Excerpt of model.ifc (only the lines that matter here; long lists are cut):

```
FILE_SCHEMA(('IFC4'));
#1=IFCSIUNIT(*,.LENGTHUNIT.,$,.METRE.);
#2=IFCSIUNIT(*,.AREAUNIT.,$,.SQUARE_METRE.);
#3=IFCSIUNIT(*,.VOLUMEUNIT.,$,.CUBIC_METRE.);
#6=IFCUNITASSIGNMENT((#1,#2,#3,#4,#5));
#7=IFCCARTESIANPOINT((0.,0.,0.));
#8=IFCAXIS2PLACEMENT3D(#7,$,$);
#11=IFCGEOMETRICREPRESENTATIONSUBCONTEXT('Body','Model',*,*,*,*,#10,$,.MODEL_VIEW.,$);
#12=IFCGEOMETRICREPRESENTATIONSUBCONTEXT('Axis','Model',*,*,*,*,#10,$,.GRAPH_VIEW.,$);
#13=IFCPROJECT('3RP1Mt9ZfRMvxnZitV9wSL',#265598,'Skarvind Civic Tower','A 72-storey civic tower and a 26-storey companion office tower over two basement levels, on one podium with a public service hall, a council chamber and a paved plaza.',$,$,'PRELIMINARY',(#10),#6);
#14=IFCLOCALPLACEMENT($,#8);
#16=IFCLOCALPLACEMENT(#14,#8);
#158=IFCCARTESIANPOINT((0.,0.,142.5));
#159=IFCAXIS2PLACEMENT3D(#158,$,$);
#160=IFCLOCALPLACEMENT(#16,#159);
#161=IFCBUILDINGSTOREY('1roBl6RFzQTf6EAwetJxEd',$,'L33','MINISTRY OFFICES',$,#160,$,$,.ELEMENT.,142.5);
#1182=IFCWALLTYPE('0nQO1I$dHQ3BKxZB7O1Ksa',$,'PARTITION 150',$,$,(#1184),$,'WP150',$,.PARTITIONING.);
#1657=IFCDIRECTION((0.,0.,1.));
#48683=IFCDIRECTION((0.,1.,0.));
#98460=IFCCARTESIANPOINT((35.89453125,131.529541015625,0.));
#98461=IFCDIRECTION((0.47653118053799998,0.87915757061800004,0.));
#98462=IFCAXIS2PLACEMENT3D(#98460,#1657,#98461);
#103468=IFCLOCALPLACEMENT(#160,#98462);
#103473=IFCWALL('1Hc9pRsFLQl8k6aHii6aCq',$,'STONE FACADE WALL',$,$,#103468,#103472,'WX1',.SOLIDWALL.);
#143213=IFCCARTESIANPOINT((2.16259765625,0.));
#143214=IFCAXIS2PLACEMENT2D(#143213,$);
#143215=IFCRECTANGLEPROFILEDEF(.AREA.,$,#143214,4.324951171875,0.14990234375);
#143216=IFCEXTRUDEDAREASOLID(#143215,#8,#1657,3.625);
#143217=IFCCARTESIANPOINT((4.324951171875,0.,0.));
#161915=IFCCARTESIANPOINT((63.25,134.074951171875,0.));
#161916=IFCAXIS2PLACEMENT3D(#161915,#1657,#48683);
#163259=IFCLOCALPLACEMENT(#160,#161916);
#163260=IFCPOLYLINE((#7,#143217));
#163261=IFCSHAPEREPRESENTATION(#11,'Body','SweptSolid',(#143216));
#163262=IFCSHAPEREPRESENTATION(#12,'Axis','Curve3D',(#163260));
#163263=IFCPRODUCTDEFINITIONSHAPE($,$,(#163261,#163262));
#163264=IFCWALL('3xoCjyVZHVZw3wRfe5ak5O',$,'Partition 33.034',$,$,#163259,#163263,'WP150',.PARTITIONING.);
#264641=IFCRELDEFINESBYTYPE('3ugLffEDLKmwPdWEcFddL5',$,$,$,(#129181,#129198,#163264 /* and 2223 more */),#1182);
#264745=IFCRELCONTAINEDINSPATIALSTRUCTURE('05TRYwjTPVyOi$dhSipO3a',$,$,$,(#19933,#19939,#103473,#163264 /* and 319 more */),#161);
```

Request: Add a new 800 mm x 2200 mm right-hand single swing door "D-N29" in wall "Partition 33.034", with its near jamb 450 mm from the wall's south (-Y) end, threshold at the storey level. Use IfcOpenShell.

```python
import numpy as np
import ifcopenshell
import ifcopenshell.api.feature
import ifcopenshell.api.geometry
import ifcopenshell.api.root
import ifcopenshell.api.spatial
import ifcopenshell.geom
import ifcopenshell.util.element
import ifcopenshell.util.placement
import ifcopenshell.util.representation
import ifcopenshell.util.shape
import ifcopenshell.util.unit

model = ifcopenshell.open("model.ifc")
unit_scale = ifcopenshell.util.unit.calculate_unit_scale(model)
settings = ifcopenshell.geom.settings()


def volume(element):
    """Net volume in cubic metres, openings subtracted."""
    shape = ifcopenshell.geom.create_shape(settings, element)
    return ifcopenshell.util.shape.get_volume(shape.geometry)


wall = model.by_id(163264)
storey = ifcopenshell.util.element.get_container(wall, ifc_class="IfcBuildingStorey")
context = ifcopenshell.util.representation.get_context(model, "Model", "Body", "MODEL_VIEW")
before = volume(wall)

width, height, from_end, sill = 0.8, 2.2, 0.45, 0.0  # metres

# The wall runs along its own X axis, and the end named is its -X end.
wall_shape = ifcopenshell.geom.create_shape(settings, wall)
x, y, z = ifcopenshell.util.shape.get_vertices(wall_shape.geometry).T
start = x.min() + from_end
face, thickness = float(y.min()), float(y.max() - y.min())
wall_matrix = ifcopenshell.util.placement.get_local_placement(wall.ObjectPlacement)
level = ifcopenshell.util.placement.get_local_placement(storey.ObjectPlacement)[2, 3]


def in_wall(x, y):
    """Placement at x, y metres in the wall's axes, at sill height."""
    matrix = wall_matrix.copy()
    matrix[:, 3] = wall_matrix @ np.array([x / unit_scale, y / unit_scale, 0.0, 1.0])
    matrix[2, 3] = level + sill / unit_scale
    return matrix


# Opening: a box that overshoots both wall faces by 50 mm.
opening = ifcopenshell.api.root.create_entity(model, ifc_class="IfcOpeningElement", predefined_type="OPENING")
box = ifcopenshell.api.geometry.add_wall_representation(
    model, context=context, length=width, height=height, thickness=thickness + 0.1
)
ifcopenshell.api.geometry.assign_representation(model, product=opening, representation=box)
ifcopenshell.api.geometry.edit_object_placement(model, product=opening, matrix=in_wall(start, face - 0.05), is_si=False)
ifcopenshell.api.feature.add_feature(model, feature=opening, element=wall)

door = ifcopenshell.api.root.create_entity(model, ifc_class="IfcDoor", name="D-N29", predefined_type="DOOR")
door.OverallWidth, door.OverallHeight = width / unit_scale, height / unit_scale
door.OperationType = "SINGLE_SWING_RIGHT"
body = ifcopenshell.api.geometry.add_door_representation(
    model,
    context=context,
    overall_width=door.OverallWidth,
    overall_height=door.OverallHeight,
    operation_type="SINGLE_SWING_RIGHT",
    lining_properties={"LiningDepth": thickness / unit_scale, "ThresholdDepth": thickness / unit_scale},
)
ifcopenshell.api.geometry.assign_representation(model, product=door, representation=body)
ifcopenshell.api.spatial.assign_container(model, products=[door], relating_structure=storey)
ifcopenshell.api.feature.add_filling(model, opening=opening, element=door)

# The lining spans the wall, so the door starts at the wall face.
ifcopenshell.api.geometry.edit_object_placement(model, product=door, matrix=in_wall(start, face), is_si=False)

after = volume(wall)

print(f"wall volume {before:.3f} -> {after:.3f} m3")

model.write("model_v2.ifc")
```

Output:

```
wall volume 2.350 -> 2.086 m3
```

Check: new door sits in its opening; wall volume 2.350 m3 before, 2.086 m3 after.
